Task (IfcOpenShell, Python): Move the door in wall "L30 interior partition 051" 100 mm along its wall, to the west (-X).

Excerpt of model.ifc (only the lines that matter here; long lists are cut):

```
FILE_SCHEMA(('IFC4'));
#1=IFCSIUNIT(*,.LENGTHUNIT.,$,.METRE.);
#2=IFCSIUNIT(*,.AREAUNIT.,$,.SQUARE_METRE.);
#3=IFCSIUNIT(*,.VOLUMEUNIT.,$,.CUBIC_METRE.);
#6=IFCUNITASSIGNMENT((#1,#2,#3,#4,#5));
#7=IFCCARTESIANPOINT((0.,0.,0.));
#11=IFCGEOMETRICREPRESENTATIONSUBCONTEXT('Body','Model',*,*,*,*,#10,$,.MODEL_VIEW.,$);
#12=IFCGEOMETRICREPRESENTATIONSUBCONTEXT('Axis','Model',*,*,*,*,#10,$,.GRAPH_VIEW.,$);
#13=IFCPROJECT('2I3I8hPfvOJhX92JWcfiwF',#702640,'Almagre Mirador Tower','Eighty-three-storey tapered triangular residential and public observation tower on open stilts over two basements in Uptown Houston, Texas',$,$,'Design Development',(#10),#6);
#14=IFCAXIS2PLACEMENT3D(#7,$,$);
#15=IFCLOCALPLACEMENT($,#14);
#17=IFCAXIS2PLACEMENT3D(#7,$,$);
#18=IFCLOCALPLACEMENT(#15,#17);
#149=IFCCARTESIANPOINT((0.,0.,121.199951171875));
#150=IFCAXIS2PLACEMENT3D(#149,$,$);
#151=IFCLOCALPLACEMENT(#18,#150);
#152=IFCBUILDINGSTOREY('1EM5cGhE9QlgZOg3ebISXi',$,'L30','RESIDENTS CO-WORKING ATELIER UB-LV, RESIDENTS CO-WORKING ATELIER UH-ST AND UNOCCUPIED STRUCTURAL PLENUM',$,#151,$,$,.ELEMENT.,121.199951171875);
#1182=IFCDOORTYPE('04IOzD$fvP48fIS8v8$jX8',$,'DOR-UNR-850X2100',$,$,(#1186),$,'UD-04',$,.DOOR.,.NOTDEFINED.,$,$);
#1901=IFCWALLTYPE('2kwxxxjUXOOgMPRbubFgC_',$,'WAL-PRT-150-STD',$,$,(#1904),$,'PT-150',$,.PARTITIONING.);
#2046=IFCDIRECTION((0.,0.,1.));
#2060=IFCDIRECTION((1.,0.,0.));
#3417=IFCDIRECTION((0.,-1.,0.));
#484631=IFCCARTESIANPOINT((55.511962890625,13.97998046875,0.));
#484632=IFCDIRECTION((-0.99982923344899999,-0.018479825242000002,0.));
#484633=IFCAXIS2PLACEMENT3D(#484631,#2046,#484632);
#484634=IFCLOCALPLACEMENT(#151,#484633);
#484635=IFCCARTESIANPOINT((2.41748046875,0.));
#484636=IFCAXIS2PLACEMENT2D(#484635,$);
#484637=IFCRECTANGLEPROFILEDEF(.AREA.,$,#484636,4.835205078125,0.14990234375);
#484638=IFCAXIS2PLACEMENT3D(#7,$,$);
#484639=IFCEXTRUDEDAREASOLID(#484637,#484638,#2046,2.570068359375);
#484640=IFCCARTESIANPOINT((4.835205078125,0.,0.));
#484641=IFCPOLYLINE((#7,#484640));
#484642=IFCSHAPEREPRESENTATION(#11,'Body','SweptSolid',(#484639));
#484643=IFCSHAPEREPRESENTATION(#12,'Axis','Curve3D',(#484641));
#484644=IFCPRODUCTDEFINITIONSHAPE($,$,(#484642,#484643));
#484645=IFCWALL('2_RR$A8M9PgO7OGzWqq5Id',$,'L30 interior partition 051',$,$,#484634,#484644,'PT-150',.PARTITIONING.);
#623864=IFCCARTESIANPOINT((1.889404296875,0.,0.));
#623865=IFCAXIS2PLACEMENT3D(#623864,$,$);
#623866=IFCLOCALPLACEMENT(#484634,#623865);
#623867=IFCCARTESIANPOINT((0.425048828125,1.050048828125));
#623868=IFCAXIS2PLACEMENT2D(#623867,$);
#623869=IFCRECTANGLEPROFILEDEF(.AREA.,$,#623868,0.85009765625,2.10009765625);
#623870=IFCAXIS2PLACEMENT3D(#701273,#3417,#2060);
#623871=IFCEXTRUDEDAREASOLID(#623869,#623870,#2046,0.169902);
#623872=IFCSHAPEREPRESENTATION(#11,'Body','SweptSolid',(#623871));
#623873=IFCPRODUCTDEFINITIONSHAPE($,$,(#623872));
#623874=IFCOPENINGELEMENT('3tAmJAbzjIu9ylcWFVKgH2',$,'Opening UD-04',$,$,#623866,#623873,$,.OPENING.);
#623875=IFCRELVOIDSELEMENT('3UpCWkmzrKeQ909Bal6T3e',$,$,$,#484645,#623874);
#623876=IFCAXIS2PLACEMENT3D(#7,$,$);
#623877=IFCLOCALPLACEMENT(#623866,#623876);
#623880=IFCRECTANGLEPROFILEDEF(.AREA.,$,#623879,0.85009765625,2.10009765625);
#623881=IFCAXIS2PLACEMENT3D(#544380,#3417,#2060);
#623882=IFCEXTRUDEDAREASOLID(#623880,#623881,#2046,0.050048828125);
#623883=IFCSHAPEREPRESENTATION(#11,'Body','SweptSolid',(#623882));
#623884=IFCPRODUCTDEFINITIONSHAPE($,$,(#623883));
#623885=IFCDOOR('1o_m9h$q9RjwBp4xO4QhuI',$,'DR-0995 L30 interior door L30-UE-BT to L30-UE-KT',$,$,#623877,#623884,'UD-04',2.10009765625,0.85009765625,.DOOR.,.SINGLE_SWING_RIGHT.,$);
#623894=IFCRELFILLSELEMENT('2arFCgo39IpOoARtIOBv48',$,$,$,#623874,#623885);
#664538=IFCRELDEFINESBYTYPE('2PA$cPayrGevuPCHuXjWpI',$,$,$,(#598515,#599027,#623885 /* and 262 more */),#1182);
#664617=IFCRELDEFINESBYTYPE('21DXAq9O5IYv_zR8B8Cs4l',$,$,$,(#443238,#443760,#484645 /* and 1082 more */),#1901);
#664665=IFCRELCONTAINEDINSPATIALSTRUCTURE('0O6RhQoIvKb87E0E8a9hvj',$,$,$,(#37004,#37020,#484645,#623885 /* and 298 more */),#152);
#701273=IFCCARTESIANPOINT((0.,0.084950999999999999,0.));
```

```python
import ifcopenshell
import ifcopenshell.api.geometry
import ifcopenshell.util.placement
import ifcopenshell.util.unit

model = ifcopenshell.open("model.ifc")
unit_scale = ifcopenshell.util.unit.calculate_unit_scale(model)

door = model.by_guid("1o_m9h$q9RjwBp4xO4QhuI")
opening = door.FillsVoids[0].RelatingOpeningElement
wall = opening.VoidsElements[0].RelatingBuildingElement

wall_matrix = ifcopenshell.util.placement.get_local_placement(wall.ObjectPlacement)
shift = wall_matrix[:3, 0] * 0.1 / unit_scale
before = ifcopenshell.util.placement.get_local_placement(door.ObjectPlacement)[:3, 3].copy()

# The door is placed relative to its opening, so it follows when the opening moves.
matrix = ifcopenshell.util.placement.get_local_placement(opening.ObjectPlacement)
matrix[:3, 3] += shift
ifcopenshell.api.geometry.edit_object_placement(
    model, product=opening, matrix=matrix, is_si=False, should_transform_children=True
)

after = ifcopenshell.util.placement.get_local_placement(door.ObjectPlacement)[:3, 3]
print("door moved by", (after - before).round(3) + 0.0)

model.write("model_edited.ifc")
```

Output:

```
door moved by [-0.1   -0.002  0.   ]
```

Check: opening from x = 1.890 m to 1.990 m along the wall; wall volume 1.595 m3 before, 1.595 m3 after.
